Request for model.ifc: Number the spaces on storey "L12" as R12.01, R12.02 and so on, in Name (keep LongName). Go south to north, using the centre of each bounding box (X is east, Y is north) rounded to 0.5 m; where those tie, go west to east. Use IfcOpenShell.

First a look at what the model holds.

```python
import ifcopenshell
import ifcopenshell.util.element
import ifcopenshell.util.placement

model = ifcopenshell.open("model.ifc")
print(model.schema)
storey = next(s for s in model.by_type("IfcBuildingStorey") if s.Name == "L12")
spaces = [e for e in ifcopenshell.util.element.get_decomposition(storey) if e.is_a("IfcSpace")]
for e in sorted(spaces, key=lambda e: e.id()):
    origin = ifcopenshell.util.placement.get_local_placement(e.ObjectPlacement)[:3, 3]
    print(e.id(), e.Name, e.LongName, origin.round(2) + 0.0, sep=" | ")
```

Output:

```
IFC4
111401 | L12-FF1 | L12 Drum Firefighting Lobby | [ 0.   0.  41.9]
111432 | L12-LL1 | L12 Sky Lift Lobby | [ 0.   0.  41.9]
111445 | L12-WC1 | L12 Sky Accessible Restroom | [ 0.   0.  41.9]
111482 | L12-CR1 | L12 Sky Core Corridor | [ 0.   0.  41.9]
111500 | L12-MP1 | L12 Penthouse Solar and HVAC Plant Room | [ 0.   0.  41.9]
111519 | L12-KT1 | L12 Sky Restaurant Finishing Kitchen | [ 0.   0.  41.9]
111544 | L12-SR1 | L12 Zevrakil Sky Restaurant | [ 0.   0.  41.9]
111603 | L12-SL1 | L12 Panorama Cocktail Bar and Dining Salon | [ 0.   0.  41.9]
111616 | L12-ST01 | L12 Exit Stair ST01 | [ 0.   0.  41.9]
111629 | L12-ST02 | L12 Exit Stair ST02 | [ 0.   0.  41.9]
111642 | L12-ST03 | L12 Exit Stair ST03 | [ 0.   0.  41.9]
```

```python
import ifcopenshell
import ifcopenshell.geom
import ifcopenshell.util.element
import ifcopenshell.util.shape

model = ifcopenshell.open("model.ifc")
settings = ifcopenshell.geom.settings()
settings.set("use-world-coords", True)


def centre(element):
    shape = ifcopenshell.geom.create_shape(settings, element)
    return ifcopenshell.util.shape.get_bbox_centroid(shape.geometry)


storey = next(s for s in model.by_type("IfcBuildingStorey") if s.Name == "L12")
spaces = [e for e in ifcopenshell.util.element.get_decomposition(storey) if e.is_a("IfcSpace")]

# Insertion points can sit at a corner or the storey origin, so sort by the geometry (in metres).
centres = {e: centre(e) for e in spaces}
spaces.sort(key=lambda e: (round(centres[e][1] / 0.5), centres[e][0]))

for i, e in enumerate(spaces, start=1):
    number = f"R12.{i:02d}"
    e.Name = number
    print(e.id(), number)

model.write("model_v2.ifc")
```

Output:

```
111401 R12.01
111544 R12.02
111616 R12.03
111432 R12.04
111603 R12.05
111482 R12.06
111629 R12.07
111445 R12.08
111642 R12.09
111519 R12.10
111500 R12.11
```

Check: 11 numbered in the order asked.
